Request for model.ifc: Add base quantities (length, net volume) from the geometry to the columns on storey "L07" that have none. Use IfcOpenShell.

First a look at what the model holds.

```python
import ifcopenshell
import ifcopenshell.util.element
import ifcopenshell.util.unit

model = ifcopenshell.open("model.ifc")
print(model.schema)
for unit_type in ("LENGTHUNIT", "AREAUNIT", "VOLUMEUNIT"):
    print(unit_type, ifcopenshell.util.unit.calculate_unit_scale(model, unit_type))
storey = next(s for s in model.by_type("IfcBuildingStorey") if s.Name == "L07")
columns = [e for e in ifcopenshell.util.element.get_decomposition(storey) if e.is_a("IfcColumn")]
for e in sorted(columns, key=lambda e: e.id()):
    print(e.id(), e.is_a(), e.Name, list(ifcopenshell.util.element.get_psets(e, qtos_only=True)), sep=" | ")
```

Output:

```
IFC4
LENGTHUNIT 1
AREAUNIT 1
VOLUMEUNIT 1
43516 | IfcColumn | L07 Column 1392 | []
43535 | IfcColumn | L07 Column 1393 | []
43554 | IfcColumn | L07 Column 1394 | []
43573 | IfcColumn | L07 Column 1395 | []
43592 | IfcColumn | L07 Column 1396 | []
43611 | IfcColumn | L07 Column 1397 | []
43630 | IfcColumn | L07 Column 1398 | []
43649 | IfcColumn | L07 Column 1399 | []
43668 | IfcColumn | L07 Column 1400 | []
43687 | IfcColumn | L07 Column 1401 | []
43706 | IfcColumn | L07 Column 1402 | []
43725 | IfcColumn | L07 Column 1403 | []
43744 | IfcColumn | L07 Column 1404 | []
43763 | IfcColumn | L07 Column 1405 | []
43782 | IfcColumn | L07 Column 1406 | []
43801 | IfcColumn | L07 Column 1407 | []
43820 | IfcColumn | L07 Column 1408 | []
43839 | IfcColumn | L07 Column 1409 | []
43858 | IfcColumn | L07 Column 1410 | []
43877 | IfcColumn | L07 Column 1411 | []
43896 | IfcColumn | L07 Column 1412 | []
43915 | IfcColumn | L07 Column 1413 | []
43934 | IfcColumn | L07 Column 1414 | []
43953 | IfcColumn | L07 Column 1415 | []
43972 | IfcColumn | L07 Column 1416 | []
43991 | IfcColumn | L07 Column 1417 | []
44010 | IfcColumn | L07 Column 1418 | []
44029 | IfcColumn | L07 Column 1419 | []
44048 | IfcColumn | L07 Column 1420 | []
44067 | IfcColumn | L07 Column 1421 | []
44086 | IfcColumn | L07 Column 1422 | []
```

```python
import ifcopenshell
import ifcopenshell.api.pset
import ifcopenshell.geom
import ifcopenshell.util.element
import ifcopenshell.util.shape
import ifcopenshell.util.unit

model = ifcopenshell.open("model.ifc")
unit_scale = ifcopenshell.util.unit.calculate_unit_scale(model)
volume_scale = ifcopenshell.util.unit.calculate_unit_scale(model, "VOLUMEUNIT")
settings = ifcopenshell.geom.settings()

storey = next(s for s in model.by_type("IfcBuildingStorey") if s.Name == "L07")
columns = [e for e in ifcopenshell.util.element.get_decomposition(storey) if e.is_a("IfcColumn")]

for e in sorted(columns, key=lambda e: e.id()):
    if ifcopenshell.util.element.get_psets(e, qtos_only=True, should_inherit=False):
        continue
    # Geometry comes back in metres, in the element's own axes.
    shape = ifcopenshell.geom.create_shape(settings, e)
    values = {
        "Length": ifcopenshell.util.shape.get_z(shape.geometry) / unit_scale,
        "NetVolume": ifcopenshell.util.shape.get_volume(shape.geometry) / volume_scale,
    }
    qto = ifcopenshell.api.pset.add_qto(model, product=e, name="Qto_ColumnBaseQuantities")
    ifcopenshell.api.pset.edit_qto(model, qto=qto, properties=values)
    print(e.id(), {k: round(v, 3) for k, v in values.items()})

model.write("model-out.ifc")
```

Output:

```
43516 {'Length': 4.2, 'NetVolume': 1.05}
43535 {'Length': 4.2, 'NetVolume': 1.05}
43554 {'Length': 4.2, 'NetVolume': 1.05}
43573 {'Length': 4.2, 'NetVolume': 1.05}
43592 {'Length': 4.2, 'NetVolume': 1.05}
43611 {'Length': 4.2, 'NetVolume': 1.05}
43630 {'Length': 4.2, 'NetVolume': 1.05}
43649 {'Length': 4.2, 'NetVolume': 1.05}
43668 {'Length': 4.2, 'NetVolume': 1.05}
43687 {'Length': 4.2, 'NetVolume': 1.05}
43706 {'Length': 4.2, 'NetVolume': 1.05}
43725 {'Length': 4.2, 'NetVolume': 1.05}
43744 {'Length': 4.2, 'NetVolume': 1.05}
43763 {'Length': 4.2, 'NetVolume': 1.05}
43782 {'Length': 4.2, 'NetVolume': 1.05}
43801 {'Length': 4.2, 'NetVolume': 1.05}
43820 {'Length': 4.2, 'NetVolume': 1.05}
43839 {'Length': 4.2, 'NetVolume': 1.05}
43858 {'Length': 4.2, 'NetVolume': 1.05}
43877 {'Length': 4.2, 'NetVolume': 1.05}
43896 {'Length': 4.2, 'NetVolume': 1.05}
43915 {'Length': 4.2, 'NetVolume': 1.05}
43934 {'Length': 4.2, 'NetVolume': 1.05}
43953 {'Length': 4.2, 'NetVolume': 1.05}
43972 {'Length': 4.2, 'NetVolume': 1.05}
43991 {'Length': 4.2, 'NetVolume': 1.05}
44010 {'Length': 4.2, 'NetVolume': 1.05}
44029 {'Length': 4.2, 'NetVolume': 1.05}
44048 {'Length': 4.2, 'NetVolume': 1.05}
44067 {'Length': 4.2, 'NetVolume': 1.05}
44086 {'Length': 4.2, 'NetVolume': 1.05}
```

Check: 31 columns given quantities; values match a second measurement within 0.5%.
